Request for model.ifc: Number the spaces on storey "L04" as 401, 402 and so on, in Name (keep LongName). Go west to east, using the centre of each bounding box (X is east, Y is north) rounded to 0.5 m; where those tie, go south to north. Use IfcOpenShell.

First a look at what the model holds.

```python
import ifcopenshell
import ifcopenshell.util.element
import ifcopenshell.util.placement

model = ifcopenshell.open("model.ifc")
print(model.schema)
storey = next(s for s in model.by_type("IfcBuildingStorey") if s.Name == "L04")
spaces = [e for e in ifcopenshell.util.element.get_decomposition(storey) if e.is_a("IfcSpace")]
for e in sorted(spaces, key=lambda e: e.id()):
    origin = ifcopenshell.util.placement.get_local_placement(e.ObjectPlacement)[:3, 3]
    print(e.id(), e.Name, e.LongName, origin.round(2) + 0.0, sep=" | ")
```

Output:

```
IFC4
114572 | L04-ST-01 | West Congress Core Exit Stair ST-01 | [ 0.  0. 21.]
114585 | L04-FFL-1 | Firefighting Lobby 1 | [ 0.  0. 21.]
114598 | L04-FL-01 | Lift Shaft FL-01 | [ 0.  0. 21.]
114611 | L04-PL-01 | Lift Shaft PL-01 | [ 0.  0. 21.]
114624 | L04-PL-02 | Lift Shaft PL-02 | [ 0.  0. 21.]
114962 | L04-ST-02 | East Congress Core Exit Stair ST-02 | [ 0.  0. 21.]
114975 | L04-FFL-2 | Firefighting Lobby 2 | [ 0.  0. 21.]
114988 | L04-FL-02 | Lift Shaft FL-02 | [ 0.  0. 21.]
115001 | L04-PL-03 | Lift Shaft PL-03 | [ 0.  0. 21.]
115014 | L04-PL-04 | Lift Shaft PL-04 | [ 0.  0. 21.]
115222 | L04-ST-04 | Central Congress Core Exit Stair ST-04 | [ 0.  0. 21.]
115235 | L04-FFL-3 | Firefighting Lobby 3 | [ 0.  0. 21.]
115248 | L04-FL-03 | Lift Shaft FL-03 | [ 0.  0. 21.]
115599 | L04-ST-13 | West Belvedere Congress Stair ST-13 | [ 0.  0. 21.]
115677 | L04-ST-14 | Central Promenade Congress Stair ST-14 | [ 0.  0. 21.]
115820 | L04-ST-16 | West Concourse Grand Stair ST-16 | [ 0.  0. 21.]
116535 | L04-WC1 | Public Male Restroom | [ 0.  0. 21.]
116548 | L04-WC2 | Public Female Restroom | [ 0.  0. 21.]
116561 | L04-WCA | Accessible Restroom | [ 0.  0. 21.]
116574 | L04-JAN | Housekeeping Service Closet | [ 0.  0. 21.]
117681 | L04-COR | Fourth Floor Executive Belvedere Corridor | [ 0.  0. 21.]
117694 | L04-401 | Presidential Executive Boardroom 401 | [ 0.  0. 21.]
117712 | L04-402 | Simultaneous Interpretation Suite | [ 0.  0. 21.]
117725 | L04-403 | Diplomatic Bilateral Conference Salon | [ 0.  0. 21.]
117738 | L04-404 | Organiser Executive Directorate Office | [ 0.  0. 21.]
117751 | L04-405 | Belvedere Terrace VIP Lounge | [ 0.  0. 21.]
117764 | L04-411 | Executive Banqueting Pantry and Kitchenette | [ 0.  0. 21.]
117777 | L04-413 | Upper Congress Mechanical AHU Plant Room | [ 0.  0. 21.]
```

```python
import ifcopenshell
import ifcopenshell.geom
import ifcopenshell.util.element
import ifcopenshell.util.shape

model = ifcopenshell.open("model.ifc")
settings = ifcopenshell.geom.settings()
settings.set("use-world-coords", True)


def centre(element):
    shape = ifcopenshell.geom.create_shape(settings, element)
    return ifcopenshell.util.shape.get_bbox_centroid(shape.geometry)


storey = next(s for s in model.by_type("IfcBuildingStorey") if s.Name == "L04")
spaces = [e for e in ifcopenshell.util.element.get_decomposition(storey) if e.is_a("IfcSpace")]

# Insertion points can sit at a corner or the storey origin, so sort by the geometry (in metres).
centres = {e: centre(e) for e in spaces}
spaces.sort(key=lambda e: (round(centres[e][0] / 0.5), centres[e][1]))

for i, e in enumerate(spaces, start=1):
    number = f"4{i:02d}"
    e.Name = number
    print(e.id(), number)

model.write("model_edited.ifc")
```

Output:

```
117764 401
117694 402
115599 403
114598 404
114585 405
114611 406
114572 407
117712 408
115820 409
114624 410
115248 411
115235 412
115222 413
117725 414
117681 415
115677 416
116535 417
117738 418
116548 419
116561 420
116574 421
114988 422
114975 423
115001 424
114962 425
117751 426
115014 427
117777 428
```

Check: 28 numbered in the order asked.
